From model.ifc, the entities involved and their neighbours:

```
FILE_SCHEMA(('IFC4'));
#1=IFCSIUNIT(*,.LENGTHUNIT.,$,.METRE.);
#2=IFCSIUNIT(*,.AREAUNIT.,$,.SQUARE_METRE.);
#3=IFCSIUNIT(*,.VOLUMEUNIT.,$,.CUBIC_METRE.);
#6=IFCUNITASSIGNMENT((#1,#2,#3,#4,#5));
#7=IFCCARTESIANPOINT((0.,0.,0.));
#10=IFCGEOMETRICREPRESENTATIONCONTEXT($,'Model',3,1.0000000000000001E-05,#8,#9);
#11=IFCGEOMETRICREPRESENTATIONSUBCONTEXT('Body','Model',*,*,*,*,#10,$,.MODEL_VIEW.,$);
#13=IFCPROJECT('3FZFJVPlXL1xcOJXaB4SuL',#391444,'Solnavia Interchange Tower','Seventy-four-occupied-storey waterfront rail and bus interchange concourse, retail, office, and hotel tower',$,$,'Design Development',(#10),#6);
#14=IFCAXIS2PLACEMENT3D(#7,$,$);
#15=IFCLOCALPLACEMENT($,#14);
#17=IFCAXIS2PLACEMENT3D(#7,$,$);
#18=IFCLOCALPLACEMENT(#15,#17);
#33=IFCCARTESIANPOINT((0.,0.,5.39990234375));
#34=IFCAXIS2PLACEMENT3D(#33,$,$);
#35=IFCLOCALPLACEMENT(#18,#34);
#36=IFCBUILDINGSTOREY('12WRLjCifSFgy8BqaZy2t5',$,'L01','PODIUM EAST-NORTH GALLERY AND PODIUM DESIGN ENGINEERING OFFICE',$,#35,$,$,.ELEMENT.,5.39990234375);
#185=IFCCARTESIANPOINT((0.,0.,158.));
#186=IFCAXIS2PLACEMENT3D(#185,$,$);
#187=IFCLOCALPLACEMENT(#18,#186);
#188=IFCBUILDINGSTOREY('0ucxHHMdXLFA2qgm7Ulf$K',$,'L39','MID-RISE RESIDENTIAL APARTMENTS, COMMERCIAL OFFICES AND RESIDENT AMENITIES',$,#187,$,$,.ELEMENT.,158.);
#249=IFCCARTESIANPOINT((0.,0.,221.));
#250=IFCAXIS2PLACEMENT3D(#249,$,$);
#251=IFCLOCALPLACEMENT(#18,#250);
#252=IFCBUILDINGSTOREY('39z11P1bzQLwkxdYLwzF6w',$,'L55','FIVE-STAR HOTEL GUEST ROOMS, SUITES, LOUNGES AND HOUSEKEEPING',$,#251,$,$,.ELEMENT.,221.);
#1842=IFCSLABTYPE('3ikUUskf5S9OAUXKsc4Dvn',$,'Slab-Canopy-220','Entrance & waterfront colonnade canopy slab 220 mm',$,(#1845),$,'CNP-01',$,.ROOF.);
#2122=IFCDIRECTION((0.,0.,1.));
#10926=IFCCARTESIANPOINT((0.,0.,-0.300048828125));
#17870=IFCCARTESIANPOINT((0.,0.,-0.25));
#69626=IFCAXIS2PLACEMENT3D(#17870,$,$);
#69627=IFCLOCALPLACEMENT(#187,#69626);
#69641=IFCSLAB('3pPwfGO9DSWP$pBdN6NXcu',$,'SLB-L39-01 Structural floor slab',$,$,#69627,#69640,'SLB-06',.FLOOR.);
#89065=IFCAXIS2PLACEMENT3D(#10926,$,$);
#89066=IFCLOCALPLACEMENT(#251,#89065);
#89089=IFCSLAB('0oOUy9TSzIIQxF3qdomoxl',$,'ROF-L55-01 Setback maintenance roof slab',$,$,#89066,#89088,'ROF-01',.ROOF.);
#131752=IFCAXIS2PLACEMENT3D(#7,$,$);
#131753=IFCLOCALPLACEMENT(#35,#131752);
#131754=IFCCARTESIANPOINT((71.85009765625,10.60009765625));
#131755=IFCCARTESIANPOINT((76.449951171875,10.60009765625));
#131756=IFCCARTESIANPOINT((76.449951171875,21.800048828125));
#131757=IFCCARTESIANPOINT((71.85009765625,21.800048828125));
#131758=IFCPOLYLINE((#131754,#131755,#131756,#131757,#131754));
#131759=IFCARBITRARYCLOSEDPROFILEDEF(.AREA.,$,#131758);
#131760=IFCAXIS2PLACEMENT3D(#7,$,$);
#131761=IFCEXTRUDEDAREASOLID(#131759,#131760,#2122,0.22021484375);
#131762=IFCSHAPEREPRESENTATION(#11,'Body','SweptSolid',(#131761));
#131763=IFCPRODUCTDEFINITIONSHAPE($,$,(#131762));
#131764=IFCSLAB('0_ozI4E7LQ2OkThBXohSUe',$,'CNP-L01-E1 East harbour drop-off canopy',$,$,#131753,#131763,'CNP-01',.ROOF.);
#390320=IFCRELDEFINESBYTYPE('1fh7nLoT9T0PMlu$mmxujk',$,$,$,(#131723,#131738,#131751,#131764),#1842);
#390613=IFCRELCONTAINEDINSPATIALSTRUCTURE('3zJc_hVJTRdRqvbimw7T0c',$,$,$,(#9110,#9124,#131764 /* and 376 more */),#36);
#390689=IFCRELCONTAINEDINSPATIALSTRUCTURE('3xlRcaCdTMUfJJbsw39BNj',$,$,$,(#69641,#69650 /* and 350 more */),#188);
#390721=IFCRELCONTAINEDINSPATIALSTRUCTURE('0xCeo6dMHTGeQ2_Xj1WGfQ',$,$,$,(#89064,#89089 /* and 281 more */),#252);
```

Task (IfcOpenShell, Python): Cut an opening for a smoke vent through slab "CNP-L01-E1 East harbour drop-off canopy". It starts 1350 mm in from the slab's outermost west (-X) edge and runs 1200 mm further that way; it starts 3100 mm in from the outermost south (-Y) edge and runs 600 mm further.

```python
import numpy as np
import ifcopenshell
import ifcopenshell.api.feature
import ifcopenshell.api.geometry
import ifcopenshell.api.root
import ifcopenshell.geom
import ifcopenshell.util.placement
import ifcopenshell.util.representation
import ifcopenshell.util.shape
import ifcopenshell.util.unit

model = ifcopenshell.open("model.ifc")
unit_scale = ifcopenshell.util.unit.calculate_unit_scale(model)
settings = ifcopenshell.geom.settings()


def volume(element):
    """Net volume in cubic metres, openings subtracted."""
    shape = ifcopenshell.geom.create_shape(settings, element)
    return ifcopenshell.util.shape.get_volume(shape.geometry)


slab = model.by_guid("0_ozI4E7LQ2OkThBXohSUe")
before = volume(slab)

# Extent in the slab's own axes, in metres. The edges named are its -X and -Y sides.
slab_shape = ifcopenshell.geom.create_shape(settings, slab)
vertices = ifcopenshell.util.shape.get_vertices(slab_shape.geometry)
x_min, y_min, bottom = vertices.min(axis=0)
top = vertices[:, 2].max()

opening = ifcopenshell.api.root.create_entity(model, ifc_class="IfcOpeningElement", name="Smoke vent opening", predefined_type="OPENING")
context = ifcopenshell.util.representation.get_context(model, "Model", "Body", "MODEL_VIEW")
width, depth = 1.2, 0.6
outline = [(0.0, 0.0), (width, 0.0), (width, depth), (0.0, depth), (0.0, 0.0)]
# Overshoot both faces by 50 mm so the cut is clean.
shape = ifcopenshell.api.geometry.add_slab_representation(
    model, context=context, depth=top - bottom + 0.1, polyline=outline
)
ifcopenshell.api.geometry.assign_representation(model, product=opening, representation=shape)

matrix = ifcopenshell.util.placement.get_local_placement(slab.ObjectPlacement)
matrix[:, 3] = matrix @ np.append(np.array([x_min + 1.35, y_min + 3.1, bottom - 0.05]) / unit_scale, 1.0)
ifcopenshell.api.geometry.edit_object_placement(model, product=opening, matrix=matrix, is_si=False)
ifcopenshell.api.feature.add_feature(model, feature=opening, element=slab)

after = volume(slab)

print(f"slab volume {before:.3f} -> {after:.3f} m3")

model.write("model_updated.ifc")
```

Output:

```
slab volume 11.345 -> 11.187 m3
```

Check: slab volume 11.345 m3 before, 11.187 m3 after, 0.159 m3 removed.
